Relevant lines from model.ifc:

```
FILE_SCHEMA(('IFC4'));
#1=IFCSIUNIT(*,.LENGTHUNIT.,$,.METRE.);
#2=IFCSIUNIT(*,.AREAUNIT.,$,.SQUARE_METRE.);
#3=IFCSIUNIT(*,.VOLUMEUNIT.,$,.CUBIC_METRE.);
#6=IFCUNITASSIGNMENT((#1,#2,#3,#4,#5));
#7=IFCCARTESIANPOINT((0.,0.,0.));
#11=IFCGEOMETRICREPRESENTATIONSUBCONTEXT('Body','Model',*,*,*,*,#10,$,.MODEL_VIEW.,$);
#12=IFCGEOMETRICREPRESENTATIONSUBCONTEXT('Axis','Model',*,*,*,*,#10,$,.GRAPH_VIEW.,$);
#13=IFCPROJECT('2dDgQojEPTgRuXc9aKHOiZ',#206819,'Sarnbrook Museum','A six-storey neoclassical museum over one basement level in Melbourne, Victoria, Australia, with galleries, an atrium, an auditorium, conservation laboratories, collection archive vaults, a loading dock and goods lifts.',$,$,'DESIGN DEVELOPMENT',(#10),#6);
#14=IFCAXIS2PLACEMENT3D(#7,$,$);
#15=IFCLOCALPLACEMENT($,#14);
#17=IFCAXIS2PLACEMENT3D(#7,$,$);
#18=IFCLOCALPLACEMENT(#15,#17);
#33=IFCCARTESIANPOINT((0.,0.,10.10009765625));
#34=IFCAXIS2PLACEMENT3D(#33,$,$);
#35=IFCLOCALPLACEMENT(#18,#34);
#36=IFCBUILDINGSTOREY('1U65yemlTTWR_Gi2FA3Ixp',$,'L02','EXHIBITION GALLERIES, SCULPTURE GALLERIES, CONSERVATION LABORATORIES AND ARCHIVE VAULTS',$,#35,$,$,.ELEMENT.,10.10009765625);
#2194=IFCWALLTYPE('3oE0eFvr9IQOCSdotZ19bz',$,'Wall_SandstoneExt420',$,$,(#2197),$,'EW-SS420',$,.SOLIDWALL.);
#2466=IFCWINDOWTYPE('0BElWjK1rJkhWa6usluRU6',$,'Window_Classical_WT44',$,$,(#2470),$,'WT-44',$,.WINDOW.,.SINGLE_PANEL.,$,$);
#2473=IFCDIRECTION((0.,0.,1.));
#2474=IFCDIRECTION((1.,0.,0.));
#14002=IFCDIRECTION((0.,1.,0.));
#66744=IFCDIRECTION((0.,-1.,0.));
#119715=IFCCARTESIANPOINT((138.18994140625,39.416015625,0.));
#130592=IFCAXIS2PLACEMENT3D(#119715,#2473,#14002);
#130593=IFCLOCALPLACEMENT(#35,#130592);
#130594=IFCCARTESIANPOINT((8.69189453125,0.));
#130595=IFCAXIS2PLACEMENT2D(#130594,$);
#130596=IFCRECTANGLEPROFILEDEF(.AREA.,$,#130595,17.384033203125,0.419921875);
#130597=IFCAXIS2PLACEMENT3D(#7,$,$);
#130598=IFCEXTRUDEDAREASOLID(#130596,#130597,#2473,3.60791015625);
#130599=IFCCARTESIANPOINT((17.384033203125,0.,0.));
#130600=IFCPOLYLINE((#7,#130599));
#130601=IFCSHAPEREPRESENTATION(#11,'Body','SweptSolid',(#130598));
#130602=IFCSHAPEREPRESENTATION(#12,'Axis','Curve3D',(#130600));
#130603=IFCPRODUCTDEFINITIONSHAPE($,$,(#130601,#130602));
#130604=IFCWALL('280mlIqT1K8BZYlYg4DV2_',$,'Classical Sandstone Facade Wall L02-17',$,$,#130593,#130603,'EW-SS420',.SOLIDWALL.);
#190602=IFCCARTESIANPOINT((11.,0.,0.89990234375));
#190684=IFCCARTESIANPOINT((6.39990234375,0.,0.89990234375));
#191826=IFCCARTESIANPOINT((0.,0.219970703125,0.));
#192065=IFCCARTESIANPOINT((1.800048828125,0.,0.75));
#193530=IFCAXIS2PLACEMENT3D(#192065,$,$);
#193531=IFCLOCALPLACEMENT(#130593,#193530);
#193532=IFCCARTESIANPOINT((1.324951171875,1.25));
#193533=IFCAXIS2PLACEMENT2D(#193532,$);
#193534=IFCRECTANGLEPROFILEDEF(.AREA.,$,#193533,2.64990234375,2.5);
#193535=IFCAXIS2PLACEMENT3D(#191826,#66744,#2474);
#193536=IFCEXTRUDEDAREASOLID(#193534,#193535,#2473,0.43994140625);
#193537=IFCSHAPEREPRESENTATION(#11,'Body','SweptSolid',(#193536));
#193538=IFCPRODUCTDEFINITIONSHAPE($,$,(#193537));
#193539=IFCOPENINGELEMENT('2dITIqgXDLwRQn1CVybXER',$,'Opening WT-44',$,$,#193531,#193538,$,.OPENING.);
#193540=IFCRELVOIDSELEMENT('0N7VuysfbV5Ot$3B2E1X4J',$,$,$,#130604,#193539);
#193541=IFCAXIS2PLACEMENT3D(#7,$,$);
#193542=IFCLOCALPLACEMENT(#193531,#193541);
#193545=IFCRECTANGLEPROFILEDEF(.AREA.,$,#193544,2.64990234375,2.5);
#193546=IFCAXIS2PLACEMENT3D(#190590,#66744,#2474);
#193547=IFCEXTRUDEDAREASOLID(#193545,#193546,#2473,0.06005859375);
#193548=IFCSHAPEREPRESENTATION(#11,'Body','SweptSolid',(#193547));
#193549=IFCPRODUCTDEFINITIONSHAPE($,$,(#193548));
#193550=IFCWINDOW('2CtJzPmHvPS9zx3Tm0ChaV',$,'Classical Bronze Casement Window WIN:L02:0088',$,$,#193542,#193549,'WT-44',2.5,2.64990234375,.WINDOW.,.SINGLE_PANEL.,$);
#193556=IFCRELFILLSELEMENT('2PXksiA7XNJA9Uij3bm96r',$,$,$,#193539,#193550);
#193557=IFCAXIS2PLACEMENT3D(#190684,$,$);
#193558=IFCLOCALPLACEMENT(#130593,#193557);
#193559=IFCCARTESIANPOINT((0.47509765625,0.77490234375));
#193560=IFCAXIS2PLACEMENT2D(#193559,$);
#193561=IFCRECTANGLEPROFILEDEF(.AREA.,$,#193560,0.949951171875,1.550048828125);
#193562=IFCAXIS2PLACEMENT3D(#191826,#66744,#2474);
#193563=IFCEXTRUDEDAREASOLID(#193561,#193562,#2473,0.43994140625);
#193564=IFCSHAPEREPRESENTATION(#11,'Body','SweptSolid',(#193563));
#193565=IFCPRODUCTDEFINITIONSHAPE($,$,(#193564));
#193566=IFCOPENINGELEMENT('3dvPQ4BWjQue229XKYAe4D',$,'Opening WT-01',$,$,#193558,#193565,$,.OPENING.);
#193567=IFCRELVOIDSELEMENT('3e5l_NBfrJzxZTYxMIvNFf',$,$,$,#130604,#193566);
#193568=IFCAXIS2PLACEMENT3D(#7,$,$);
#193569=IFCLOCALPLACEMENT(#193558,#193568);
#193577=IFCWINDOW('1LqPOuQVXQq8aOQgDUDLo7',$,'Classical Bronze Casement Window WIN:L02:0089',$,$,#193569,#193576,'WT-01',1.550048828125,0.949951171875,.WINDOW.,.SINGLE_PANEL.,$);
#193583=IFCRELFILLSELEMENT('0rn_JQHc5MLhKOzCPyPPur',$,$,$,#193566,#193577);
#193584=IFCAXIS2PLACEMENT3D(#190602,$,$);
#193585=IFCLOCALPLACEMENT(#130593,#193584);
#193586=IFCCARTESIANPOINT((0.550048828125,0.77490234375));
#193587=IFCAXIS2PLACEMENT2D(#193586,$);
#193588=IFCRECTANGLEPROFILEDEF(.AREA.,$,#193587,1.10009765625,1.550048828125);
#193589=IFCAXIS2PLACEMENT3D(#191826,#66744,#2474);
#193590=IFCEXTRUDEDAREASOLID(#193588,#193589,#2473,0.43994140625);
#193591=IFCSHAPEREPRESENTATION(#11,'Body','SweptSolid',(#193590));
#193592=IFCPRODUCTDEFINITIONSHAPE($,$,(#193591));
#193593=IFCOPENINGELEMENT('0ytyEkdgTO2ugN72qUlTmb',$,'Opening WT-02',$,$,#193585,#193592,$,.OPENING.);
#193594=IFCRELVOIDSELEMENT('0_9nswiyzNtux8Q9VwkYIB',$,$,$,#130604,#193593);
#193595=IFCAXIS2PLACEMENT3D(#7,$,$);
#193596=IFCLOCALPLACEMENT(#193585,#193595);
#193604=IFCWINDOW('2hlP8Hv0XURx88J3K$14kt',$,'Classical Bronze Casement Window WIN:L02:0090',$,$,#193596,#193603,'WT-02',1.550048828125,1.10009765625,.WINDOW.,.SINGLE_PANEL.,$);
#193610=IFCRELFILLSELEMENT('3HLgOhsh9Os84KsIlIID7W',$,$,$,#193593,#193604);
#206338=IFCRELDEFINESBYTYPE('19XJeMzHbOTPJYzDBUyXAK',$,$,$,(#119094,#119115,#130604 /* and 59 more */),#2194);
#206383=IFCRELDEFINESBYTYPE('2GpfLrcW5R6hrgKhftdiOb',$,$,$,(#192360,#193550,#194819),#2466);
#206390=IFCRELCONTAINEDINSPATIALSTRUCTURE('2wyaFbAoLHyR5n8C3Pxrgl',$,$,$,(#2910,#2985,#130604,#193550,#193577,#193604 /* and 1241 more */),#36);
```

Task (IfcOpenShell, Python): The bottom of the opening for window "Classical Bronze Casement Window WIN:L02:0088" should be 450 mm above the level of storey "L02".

```python
import numpy as np
import ifcopenshell
import ifcopenshell.api.geometry
import ifcopenshell.geom
import ifcopenshell.util.element
import ifcopenshell.util.placement
import ifcopenshell.util.shape
import ifcopenshell.util.unit

model = ifcopenshell.open("model.ifc")
unit_scale = ifcopenshell.util.unit.calculate_unit_scale(model)

window = model.by_guid("2CtJzPmHvPS9zx3Tm0ChaV")
opening = window.FillsVoids[0].RelatingOpeningElement
storey = ifcopenshell.util.element.get_container(window, ifc_class="IfcBuildingStorey")
level = ifcopenshell.util.placement.get_local_placement(storey.ObjectPlacement)[2, 3]

# The opening's origin need not be at the sill, so measure its lowest point.
shape = ifcopenshell.geom.create_shape(ifcopenshell.geom.settings(), opening)
bottom = ifcopenshell.util.shape.get_shape_bottom_elevation(shape, shape.geometry) / unit_scale
dz = level + 0.45 / unit_scale - bottom

shift = np.array([0.0, 0.0, dz])
# The window is placed relative to its opening, so it follows when the opening moves.
matrix = ifcopenshell.util.placement.get_local_placement(opening.ObjectPlacement)
matrix[:3, 3] += shift
ifcopenshell.api.geometry.edit_object_placement(
    model, product=opening, matrix=matrix, is_si=False, should_transform_children=True
)

print(f"moved by {dz * unit_scale:+.3f} m")

model.write("model_rev.ifc")
```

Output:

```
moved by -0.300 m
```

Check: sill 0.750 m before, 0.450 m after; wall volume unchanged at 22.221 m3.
